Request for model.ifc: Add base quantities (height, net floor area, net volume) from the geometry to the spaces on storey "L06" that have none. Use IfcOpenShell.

First a look at what the model holds.

```python
import ifcopenshell
import ifcopenshell.util.element
import ifcopenshell.util.unit

model = ifcopenshell.open("model.ifc")
print(model.schema)
for unit_type in ("LENGTHUNIT", "AREAUNIT", "VOLUMEUNIT"):
    print(unit_type, ifcopenshell.util.unit.calculate_unit_scale(model, unit_type))
storey = next(s for s in model.by_type("IfcBuildingStorey") if s.Name == "L06")
spaces = [e for e in ifcopenshell.util.element.get_decomposition(storey) if e.is_a("IfcSpace")]
for e in sorted(spaces, key=lambda e: e.id()):
    print(e.id(), e.is_a(), e.Name, list(ifcopenshell.util.element.get_psets(e, qtos_only=True)), sep=" | ")
```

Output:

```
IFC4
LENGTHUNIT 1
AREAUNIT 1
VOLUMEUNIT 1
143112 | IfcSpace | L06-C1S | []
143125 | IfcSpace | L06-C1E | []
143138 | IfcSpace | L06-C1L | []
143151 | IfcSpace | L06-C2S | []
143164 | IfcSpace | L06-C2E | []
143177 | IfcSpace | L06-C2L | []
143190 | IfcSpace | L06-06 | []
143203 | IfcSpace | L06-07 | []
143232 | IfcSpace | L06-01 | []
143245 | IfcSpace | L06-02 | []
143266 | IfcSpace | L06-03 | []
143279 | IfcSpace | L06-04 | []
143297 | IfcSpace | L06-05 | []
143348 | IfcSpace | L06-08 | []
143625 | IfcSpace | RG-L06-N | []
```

```python
import ifcopenshell
import ifcopenshell.api.pset
import ifcopenshell.geom
import ifcopenshell.util.element
import ifcopenshell.util.shape
import ifcopenshell.util.unit

model = ifcopenshell.open("model.ifc")
unit_scale = ifcopenshell.util.unit.calculate_unit_scale(model)
area_scale = ifcopenshell.util.unit.calculate_unit_scale(model, "AREAUNIT")
volume_scale = ifcopenshell.util.unit.calculate_unit_scale(model, "VOLUMEUNIT")
settings = ifcopenshell.geom.settings()

storey = next(s for s in model.by_type("IfcBuildingStorey") if s.Name == "L06")
spaces = [e for e in ifcopenshell.util.element.get_decomposition(storey) if e.is_a("IfcSpace")]

for e in sorted(spaces, key=lambda e: e.id()):
    if ifcopenshell.util.element.get_psets(e, qtos_only=True, should_inherit=False):
        continue
    # Geometry comes back in metres, in the element's own axes.
    shape = ifcopenshell.geom.create_shape(settings, e)
    values = {
        "Height": ifcopenshell.util.shape.get_z(shape.geometry) / unit_scale,
        "NetFloorArea": ifcopenshell.util.shape.get_footprint_area(shape.geometry) / area_scale,
        "NetVolume": ifcopenshell.util.shape.get_volume(shape.geometry) / volume_scale,
    }
    qto = ifcopenshell.api.pset.add_qto(model, product=e, name="Qto_SpaceBaseQuantities")
    ifcopenshell.api.pset.edit_qto(model, qto=qto, properties=values)
    print(e.id(), {k: round(v, 3) for k, v in values.items()})

model.write("model_rev.ifc")
```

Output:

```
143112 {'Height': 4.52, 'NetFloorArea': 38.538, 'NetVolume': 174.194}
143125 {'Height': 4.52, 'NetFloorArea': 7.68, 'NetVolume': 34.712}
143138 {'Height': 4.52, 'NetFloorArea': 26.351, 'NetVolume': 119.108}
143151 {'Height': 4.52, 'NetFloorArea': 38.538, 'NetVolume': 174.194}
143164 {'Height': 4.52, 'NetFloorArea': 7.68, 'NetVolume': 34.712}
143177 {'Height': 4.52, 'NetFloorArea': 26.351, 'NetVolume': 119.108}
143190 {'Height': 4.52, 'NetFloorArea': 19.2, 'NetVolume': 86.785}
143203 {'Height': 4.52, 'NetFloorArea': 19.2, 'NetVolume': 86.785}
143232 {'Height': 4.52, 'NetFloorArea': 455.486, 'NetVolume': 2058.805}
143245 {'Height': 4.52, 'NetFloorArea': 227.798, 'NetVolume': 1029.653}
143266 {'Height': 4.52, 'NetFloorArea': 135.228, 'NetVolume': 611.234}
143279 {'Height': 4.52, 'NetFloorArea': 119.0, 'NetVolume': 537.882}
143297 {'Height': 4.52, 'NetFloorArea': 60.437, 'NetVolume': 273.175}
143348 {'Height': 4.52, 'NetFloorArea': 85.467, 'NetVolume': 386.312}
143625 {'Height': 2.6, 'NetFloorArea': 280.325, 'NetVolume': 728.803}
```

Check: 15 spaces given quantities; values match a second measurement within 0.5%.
